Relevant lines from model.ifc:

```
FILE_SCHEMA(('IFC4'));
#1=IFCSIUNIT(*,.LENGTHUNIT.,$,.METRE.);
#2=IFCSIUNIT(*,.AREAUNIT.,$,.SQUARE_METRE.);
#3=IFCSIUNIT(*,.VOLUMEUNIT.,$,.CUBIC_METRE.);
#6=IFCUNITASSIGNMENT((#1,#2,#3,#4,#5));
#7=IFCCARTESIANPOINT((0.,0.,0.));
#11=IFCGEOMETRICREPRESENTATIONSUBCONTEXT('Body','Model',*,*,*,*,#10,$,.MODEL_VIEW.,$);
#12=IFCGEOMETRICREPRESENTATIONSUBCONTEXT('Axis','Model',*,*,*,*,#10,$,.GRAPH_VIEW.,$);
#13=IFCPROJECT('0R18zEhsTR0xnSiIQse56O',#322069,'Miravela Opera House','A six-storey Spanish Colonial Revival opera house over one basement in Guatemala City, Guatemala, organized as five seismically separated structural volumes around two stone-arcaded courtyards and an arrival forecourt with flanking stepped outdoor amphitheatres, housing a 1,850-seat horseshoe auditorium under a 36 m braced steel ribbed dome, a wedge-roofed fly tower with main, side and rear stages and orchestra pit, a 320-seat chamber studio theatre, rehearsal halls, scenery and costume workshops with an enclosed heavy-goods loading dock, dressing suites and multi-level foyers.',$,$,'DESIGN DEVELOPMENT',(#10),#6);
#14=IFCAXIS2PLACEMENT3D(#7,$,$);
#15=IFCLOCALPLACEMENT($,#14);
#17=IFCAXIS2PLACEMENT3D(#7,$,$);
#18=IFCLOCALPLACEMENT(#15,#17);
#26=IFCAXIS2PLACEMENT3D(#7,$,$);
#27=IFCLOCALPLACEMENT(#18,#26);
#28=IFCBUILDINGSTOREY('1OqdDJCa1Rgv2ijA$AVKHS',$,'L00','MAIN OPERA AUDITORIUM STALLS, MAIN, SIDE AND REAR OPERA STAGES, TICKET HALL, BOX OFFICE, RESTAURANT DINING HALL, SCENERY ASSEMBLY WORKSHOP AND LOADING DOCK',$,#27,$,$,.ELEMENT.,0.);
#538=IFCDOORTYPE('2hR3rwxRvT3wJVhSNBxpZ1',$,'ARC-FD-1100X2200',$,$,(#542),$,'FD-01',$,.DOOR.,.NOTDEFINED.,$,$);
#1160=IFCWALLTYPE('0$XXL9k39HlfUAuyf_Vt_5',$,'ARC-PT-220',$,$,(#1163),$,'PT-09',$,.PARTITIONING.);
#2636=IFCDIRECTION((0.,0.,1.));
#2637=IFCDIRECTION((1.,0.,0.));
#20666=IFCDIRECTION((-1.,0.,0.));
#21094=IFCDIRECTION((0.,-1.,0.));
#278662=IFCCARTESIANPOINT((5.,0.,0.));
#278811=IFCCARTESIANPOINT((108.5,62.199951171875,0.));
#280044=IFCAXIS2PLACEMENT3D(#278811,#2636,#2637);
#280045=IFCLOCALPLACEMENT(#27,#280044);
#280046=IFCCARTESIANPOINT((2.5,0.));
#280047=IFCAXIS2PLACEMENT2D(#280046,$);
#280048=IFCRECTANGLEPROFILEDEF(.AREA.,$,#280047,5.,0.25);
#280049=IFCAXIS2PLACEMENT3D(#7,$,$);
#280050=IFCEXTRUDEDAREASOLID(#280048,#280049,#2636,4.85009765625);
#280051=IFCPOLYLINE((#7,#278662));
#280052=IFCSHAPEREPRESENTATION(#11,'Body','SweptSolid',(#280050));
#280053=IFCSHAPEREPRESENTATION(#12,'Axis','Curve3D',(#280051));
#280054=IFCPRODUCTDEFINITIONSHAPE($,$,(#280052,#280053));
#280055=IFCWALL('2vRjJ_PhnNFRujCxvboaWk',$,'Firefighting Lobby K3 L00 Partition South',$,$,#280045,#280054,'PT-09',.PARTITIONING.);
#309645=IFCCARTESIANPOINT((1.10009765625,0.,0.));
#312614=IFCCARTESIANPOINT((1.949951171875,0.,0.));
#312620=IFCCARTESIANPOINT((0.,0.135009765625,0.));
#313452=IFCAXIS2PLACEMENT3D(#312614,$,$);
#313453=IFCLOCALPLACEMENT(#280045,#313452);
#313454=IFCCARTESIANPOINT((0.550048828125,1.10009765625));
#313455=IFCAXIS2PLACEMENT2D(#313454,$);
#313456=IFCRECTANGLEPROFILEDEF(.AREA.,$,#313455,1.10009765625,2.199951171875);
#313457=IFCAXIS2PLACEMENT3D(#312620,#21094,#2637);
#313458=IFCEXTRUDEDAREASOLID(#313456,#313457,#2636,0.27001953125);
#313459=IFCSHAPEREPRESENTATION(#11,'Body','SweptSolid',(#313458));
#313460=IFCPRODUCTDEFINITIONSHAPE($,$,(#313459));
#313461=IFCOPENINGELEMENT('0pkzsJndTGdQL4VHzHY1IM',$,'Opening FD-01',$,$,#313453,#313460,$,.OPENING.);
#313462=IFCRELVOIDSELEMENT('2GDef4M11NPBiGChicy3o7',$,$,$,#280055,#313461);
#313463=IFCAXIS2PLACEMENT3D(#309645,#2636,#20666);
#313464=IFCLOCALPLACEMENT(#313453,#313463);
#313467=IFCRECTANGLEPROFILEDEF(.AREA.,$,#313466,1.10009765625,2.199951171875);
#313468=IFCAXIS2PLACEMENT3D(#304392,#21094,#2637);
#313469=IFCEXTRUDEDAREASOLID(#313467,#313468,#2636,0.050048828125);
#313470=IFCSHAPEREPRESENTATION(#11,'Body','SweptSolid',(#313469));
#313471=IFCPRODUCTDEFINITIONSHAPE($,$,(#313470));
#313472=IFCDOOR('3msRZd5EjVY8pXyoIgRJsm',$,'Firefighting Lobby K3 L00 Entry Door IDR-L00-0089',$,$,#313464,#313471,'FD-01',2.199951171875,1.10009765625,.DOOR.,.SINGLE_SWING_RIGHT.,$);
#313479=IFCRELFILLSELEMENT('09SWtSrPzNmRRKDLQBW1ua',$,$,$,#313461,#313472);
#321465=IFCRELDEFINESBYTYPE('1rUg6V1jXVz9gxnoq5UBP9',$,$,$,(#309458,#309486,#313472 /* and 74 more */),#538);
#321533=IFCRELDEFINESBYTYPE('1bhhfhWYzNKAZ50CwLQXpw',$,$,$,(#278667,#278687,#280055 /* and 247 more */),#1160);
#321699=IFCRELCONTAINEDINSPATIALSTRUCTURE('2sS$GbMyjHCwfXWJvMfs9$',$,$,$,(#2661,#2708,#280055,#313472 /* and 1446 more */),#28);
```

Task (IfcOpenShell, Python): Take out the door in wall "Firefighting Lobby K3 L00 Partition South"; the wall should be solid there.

```python
import ifcopenshell
import ifcopenshell.api.feature
import ifcopenshell.api.root
import ifcopenshell.geom
import ifcopenshell.util.shape

model = ifcopenshell.open("model.ifc")
settings = ifcopenshell.geom.settings()


def volume(element):
    """Net volume in cubic metres, openings subtracted."""
    shape = ifcopenshell.geom.create_shape(settings, element)
    return ifcopenshell.util.shape.get_volume(shape.geometry)


door = model.by_guid("3msRZd5EjVY8pXyoIgRJsm")
opening = door.FillsVoids[0].RelatingOpeningElement
wall = opening.VoidsElements[0].RelatingBuildingElement
before = volume(wall)

ifcopenshell.api.root.remove_product(model, product=door)
ifcopenshell.api.feature.remove_feature(model, feature=opening)

after = volume(wall)

print(f"wall volume {before:.3f} -> {after:.3f} m3")

model.write("model_rev.ifc")
```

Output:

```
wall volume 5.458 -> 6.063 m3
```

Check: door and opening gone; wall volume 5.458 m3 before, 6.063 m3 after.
